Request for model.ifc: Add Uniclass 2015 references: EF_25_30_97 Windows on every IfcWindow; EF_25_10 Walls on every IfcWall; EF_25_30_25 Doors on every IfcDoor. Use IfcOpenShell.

First a look at what the model holds.

```python
import ifcopenshell

model = ifcopenshell.open("model.ifc")
print(model.schema)
print("classifications:", [c.Name for c in model.by_type("IfcClassification")])
for ifc_class in ("IfcDoor", "IfcRoof", "IfcStair", "IfcWall", "IfcWindow"):
    print(ifc_class, len(model.by_type(ifc_class)))
```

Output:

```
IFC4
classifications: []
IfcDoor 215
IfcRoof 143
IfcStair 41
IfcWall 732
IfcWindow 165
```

```python
import ifcopenshell
import ifcopenshell.api.classification

model = ifcopenshell.open("model.ifc")

system = ifcopenshell.api.classification.add_classification(model, classification="Uniclass 2015")

codes = {
    "IfcWindow": ("EF_25_30_97", "Windows"),
    "IfcWall": ("EF_25_10", "Walls"),
    "IfcDoor": ("EF_25_30_25", "Doors"),
}
for ifc_class, (code, name) in codes.items():
    products = model.by_type(ifc_class)
    ifcopenshell.api.classification.add_reference(
        model, products=products, classification=system, identification=code, name=name
    )
    print(code, len(products))

model.write("model_edited.ifc")
```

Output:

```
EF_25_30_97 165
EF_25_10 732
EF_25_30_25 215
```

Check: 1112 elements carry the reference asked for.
